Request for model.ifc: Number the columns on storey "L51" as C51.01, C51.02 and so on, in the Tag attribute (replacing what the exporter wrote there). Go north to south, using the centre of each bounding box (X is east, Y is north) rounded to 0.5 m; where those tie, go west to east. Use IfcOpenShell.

First a look at what the model holds.

```python
import ifcopenshell
import ifcopenshell.util.element
import ifcopenshell.util.placement

model = ifcopenshell.open("model.ifc")
print(model.schema)
storey = next(s for s in model.by_type("IfcBuildingStorey") if s.Name == "L51")
columns = [e for e in ifcopenshell.util.element.get_decomposition(storey) if e.is_a("IfcColumn")]
for e in sorted(columns, key=lambda e: e.id()):
    origin = ifcopenshell.util.placement.get_local_placement(e.ObjectPlacement)[:3, 3]
    print(e.id(), e.Tag, e.Name, origin.round(2) + 0.0, sep=" | ")
```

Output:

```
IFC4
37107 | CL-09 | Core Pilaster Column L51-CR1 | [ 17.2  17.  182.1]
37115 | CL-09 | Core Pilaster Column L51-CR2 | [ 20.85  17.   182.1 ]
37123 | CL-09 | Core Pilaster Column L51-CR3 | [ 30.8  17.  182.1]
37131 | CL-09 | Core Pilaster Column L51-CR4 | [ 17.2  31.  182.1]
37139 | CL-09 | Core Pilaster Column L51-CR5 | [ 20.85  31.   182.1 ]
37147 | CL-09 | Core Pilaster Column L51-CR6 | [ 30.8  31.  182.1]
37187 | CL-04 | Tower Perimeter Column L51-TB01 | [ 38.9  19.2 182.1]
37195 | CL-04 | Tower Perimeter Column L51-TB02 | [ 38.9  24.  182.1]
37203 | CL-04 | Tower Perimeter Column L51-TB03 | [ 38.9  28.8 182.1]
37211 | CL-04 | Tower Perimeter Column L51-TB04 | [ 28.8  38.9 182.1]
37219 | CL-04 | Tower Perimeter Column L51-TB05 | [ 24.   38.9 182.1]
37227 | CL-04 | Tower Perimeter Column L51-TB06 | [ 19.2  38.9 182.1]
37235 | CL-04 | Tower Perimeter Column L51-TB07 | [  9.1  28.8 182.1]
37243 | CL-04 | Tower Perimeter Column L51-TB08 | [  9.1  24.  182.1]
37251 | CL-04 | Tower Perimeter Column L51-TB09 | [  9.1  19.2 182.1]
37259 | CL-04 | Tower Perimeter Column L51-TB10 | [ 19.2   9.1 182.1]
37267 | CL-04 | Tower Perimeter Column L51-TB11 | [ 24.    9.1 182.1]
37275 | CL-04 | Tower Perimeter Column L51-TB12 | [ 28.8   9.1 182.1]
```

```python
import ifcopenshell
import ifcopenshell.geom
import ifcopenshell.util.element
import ifcopenshell.util.shape

model = ifcopenshell.open("model.ifc")
settings = ifcopenshell.geom.settings()
settings.set("use-world-coords", True)


def centre(element):
    shape = ifcopenshell.geom.create_shape(settings, element)
    return ifcopenshell.util.shape.get_bbox_centroid(shape.geometry)


storey = next(s for s in model.by_type("IfcBuildingStorey") if s.Name == "L51")
columns = [e for e in ifcopenshell.util.element.get_decomposition(storey) if e.is_a("IfcColumn")]

# Insertion points can sit at a corner or the storey origin, so sort by the geometry (in metres).
centres = {e: centre(e) for e in columns}
columns.sort(key=lambda e: (-round(centres[e][1] / 0.5), centres[e][0]))

for i, e in enumerate(columns, start=1):
    number = f"C51.{i:02d}"
    e.Tag = number
    print(e.id(), number)

model.write("model-out.ifc")
```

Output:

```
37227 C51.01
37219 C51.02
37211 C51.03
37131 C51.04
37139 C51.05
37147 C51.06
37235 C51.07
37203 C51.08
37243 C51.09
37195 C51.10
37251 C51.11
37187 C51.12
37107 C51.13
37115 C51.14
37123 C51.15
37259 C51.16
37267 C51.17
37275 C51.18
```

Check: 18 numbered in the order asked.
